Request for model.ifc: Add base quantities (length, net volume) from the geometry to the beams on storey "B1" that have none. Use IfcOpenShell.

First a look at what the model holds.

```python
import ifcopenshell
import ifcopenshell.util.element
import ifcopenshell.util.unit

model = ifcopenshell.open("model.ifc")
print(model.schema)
for unit_type in ("LENGTHUNIT", "AREAUNIT", "VOLUMEUNIT"):
    print(unit_type, ifcopenshell.util.unit.calculate_unit_scale(model, unit_type))
storey = next(s for s in model.by_type("IfcBuildingStorey") if s.Name == "B1")
beams = [e for e in ifcopenshell.util.element.get_decomposition(storey) if e.is_a("IfcBeam")]
for e in sorted(beams, key=lambda e: e.id()):
    print(e.id(), e.is_a(), e.Name, list(ifcopenshell.util.element.get_psets(e, qtos_only=True)), sep=" | ")
```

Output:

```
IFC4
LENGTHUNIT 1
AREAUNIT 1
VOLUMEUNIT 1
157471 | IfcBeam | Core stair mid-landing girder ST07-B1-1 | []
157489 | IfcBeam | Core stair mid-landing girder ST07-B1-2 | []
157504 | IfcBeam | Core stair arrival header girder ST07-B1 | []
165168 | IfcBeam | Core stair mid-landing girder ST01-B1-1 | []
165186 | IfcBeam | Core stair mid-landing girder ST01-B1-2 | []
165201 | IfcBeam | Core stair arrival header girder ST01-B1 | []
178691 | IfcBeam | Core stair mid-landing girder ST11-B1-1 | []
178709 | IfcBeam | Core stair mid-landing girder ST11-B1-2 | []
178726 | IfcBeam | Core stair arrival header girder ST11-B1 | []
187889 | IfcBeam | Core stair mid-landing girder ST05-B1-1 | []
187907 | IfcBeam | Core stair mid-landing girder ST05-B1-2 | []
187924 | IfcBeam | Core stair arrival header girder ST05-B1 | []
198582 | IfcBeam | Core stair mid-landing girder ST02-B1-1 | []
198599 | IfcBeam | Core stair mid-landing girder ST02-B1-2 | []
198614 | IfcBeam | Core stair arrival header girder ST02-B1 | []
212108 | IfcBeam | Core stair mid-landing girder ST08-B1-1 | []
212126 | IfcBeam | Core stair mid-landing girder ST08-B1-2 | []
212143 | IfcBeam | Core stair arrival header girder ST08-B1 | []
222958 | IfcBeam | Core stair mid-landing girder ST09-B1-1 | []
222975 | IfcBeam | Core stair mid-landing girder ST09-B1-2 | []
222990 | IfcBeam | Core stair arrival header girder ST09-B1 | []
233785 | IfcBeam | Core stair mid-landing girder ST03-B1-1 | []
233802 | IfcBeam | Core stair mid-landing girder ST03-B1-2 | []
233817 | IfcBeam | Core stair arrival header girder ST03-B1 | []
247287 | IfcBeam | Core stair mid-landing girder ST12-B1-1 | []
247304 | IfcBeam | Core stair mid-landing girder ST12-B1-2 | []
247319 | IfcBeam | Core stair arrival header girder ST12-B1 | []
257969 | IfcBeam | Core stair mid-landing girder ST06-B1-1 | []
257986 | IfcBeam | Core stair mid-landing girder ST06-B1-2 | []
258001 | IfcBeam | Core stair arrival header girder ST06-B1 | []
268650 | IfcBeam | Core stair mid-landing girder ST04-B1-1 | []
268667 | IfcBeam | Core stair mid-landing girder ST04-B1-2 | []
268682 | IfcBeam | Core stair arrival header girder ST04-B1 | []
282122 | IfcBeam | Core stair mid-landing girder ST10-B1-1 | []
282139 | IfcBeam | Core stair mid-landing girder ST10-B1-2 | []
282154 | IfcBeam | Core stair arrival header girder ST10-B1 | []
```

```python
import ifcopenshell
import ifcopenshell.api.pset
import ifcopenshell.geom
import ifcopenshell.util.element
import ifcopenshell.util.shape
import ifcopenshell.util.unit

model = ifcopenshell.open("model.ifc")
unit_scale = ifcopenshell.util.unit.calculate_unit_scale(model)
volume_scale = ifcopenshell.util.unit.calculate_unit_scale(model, "VOLUMEUNIT")
settings = ifcopenshell.geom.settings()

storey = next(s for s in model.by_type("IfcBuildingStorey") if s.Name == "B1")
beams = [e for e in ifcopenshell.util.element.get_decomposition(storey) if e.is_a("IfcBeam")]

for e in sorted(beams, key=lambda e: e.id()):
    if ifcopenshell.util.element.get_psets(e, qtos_only=True, should_inherit=False):
        continue
    # Geometry comes back in metres, in the element's own axes.
    shape = ifcopenshell.geom.create_shape(settings, e)
    values = {
        "Length": ifcopenshell.util.shape.get_max_xyz(shape.geometry) / unit_scale,
        "NetVolume": ifcopenshell.util.shape.get_volume(shape.geometry) / volume_scale,
    }
    qto = ifcopenshell.api.pset.add_qto(model, product=e, name="Qto_BeamBaseQuantities")
    ifcopenshell.api.pset.edit_qto(model, qto=qto, properties=values)
    print(e.id(), {k: round(v, 3) for k, v in values.items()})

model.write("model_updated.ifc")
```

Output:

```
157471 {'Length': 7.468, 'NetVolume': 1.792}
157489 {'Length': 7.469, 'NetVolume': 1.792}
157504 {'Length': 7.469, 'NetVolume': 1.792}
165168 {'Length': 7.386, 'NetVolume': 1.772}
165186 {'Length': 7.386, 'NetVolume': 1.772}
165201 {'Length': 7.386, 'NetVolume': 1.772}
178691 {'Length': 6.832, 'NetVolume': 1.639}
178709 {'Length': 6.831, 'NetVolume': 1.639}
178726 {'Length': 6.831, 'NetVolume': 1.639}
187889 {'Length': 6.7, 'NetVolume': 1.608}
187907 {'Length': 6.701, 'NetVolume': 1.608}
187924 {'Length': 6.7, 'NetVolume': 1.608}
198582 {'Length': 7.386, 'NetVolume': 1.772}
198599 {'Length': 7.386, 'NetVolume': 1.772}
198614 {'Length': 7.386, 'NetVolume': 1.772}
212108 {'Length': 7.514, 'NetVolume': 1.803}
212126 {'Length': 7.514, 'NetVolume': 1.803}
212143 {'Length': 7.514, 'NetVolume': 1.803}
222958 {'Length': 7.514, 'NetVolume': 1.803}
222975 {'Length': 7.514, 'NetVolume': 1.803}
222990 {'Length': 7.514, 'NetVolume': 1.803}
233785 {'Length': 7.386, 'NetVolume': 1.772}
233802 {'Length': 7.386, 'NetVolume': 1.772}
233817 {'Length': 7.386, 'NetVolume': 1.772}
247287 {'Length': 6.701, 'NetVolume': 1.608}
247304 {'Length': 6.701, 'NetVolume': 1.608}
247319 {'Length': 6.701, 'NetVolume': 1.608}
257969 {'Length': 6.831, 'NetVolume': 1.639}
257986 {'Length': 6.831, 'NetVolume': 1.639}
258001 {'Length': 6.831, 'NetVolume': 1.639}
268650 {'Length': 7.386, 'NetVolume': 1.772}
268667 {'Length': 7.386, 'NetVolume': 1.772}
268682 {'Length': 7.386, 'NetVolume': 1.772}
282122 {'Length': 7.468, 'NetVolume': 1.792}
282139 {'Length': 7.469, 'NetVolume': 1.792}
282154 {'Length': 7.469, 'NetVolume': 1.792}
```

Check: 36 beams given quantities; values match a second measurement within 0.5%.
